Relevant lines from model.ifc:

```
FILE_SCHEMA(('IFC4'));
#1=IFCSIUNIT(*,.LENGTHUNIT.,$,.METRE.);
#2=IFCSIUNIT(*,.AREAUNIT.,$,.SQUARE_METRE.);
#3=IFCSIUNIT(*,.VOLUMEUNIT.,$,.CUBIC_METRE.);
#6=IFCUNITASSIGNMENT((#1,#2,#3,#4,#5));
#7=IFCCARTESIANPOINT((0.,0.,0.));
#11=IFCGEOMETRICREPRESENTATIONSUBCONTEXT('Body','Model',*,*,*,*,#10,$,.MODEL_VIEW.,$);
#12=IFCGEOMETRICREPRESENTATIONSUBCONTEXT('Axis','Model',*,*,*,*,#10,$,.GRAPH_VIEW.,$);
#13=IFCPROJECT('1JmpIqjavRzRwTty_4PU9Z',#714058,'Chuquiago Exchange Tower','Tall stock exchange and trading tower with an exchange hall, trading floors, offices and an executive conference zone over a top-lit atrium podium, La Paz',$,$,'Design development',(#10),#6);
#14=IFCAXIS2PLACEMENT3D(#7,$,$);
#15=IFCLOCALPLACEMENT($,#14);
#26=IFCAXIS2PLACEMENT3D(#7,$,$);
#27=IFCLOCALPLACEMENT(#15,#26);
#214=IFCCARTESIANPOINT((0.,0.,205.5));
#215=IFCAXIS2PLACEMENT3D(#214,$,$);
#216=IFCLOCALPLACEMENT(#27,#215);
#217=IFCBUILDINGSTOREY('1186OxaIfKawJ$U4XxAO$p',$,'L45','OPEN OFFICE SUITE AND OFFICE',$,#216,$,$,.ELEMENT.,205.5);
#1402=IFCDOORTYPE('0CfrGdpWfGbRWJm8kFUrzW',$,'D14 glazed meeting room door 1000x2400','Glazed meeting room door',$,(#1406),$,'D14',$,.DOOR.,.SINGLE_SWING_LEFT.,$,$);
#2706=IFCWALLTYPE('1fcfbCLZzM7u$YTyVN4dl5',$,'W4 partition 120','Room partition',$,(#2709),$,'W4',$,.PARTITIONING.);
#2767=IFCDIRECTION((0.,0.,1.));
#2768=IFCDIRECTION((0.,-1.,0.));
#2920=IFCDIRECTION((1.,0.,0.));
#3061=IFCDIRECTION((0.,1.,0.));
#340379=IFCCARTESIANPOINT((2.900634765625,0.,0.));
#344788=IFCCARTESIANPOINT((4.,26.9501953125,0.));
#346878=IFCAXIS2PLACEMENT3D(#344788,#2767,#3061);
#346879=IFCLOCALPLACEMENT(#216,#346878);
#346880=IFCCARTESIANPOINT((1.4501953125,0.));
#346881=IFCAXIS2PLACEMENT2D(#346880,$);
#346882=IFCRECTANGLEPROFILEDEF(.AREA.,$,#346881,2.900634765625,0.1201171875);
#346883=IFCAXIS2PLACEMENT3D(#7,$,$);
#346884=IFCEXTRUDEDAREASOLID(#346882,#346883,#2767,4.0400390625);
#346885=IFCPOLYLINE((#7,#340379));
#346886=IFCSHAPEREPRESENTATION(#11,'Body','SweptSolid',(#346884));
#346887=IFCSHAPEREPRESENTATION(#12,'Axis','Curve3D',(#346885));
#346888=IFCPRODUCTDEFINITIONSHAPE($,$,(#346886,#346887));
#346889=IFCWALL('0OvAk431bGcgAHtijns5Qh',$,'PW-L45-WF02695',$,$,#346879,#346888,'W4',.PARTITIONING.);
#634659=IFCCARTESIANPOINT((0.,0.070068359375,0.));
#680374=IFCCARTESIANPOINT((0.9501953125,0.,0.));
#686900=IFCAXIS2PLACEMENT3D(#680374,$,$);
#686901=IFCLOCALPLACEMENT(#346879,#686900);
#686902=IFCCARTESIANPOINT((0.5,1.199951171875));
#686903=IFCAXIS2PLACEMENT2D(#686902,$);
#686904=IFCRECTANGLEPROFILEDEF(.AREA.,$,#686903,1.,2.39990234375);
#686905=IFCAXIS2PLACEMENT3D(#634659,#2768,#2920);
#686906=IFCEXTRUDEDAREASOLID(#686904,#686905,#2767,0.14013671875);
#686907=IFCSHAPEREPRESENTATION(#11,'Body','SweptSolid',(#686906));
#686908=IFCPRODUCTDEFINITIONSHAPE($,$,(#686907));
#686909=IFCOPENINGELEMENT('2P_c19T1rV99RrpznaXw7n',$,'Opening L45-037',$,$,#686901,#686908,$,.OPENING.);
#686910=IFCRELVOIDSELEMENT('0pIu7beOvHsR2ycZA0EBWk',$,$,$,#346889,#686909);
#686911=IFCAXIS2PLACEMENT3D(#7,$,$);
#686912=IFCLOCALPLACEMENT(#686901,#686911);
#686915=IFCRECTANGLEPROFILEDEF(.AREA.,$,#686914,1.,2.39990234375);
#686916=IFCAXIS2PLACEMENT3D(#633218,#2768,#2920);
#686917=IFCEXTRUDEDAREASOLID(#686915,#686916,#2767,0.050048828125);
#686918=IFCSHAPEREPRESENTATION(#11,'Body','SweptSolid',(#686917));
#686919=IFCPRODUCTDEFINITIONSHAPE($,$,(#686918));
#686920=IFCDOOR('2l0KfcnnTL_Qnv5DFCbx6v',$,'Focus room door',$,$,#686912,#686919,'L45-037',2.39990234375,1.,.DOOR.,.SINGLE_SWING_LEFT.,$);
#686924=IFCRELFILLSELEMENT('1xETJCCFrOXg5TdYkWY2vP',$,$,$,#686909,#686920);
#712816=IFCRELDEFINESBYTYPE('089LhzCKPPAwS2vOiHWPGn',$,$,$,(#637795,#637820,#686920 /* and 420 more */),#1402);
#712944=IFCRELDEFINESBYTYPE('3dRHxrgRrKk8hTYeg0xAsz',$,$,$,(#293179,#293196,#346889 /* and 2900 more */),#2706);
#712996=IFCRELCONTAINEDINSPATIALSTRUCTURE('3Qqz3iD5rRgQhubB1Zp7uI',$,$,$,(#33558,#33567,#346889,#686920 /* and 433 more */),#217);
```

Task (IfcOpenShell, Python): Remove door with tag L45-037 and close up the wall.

```python
import ifcopenshell
import ifcopenshell.api.feature
import ifcopenshell.api.root
import ifcopenshell.geom
import ifcopenshell.util.shape

model = ifcopenshell.open("model.ifc")
settings = ifcopenshell.geom.settings()


def volume(element):
    """Net volume in cubic metres, openings subtracted."""
    shape = ifcopenshell.geom.create_shape(settings, element)
    return ifcopenshell.util.shape.get_volume(shape.geometry)


door = model.by_guid("2l0KfcnnTL_Qnv5DFCbx6v")
opening = door.FillsVoids[0].RelatingOpeningElement
wall = opening.VoidsElements[0].RelatingBuildingElement
before = volume(wall)

ifcopenshell.api.root.remove_product(model, product=door)
ifcopenshell.api.feature.remove_feature(model, feature=opening)

after = volume(wall)

print(f"wall volume {before:.3f} -> {after:.3f} m3")

model.write("model_edited.ifc")
```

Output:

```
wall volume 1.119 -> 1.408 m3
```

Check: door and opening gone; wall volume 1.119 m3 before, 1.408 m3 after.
